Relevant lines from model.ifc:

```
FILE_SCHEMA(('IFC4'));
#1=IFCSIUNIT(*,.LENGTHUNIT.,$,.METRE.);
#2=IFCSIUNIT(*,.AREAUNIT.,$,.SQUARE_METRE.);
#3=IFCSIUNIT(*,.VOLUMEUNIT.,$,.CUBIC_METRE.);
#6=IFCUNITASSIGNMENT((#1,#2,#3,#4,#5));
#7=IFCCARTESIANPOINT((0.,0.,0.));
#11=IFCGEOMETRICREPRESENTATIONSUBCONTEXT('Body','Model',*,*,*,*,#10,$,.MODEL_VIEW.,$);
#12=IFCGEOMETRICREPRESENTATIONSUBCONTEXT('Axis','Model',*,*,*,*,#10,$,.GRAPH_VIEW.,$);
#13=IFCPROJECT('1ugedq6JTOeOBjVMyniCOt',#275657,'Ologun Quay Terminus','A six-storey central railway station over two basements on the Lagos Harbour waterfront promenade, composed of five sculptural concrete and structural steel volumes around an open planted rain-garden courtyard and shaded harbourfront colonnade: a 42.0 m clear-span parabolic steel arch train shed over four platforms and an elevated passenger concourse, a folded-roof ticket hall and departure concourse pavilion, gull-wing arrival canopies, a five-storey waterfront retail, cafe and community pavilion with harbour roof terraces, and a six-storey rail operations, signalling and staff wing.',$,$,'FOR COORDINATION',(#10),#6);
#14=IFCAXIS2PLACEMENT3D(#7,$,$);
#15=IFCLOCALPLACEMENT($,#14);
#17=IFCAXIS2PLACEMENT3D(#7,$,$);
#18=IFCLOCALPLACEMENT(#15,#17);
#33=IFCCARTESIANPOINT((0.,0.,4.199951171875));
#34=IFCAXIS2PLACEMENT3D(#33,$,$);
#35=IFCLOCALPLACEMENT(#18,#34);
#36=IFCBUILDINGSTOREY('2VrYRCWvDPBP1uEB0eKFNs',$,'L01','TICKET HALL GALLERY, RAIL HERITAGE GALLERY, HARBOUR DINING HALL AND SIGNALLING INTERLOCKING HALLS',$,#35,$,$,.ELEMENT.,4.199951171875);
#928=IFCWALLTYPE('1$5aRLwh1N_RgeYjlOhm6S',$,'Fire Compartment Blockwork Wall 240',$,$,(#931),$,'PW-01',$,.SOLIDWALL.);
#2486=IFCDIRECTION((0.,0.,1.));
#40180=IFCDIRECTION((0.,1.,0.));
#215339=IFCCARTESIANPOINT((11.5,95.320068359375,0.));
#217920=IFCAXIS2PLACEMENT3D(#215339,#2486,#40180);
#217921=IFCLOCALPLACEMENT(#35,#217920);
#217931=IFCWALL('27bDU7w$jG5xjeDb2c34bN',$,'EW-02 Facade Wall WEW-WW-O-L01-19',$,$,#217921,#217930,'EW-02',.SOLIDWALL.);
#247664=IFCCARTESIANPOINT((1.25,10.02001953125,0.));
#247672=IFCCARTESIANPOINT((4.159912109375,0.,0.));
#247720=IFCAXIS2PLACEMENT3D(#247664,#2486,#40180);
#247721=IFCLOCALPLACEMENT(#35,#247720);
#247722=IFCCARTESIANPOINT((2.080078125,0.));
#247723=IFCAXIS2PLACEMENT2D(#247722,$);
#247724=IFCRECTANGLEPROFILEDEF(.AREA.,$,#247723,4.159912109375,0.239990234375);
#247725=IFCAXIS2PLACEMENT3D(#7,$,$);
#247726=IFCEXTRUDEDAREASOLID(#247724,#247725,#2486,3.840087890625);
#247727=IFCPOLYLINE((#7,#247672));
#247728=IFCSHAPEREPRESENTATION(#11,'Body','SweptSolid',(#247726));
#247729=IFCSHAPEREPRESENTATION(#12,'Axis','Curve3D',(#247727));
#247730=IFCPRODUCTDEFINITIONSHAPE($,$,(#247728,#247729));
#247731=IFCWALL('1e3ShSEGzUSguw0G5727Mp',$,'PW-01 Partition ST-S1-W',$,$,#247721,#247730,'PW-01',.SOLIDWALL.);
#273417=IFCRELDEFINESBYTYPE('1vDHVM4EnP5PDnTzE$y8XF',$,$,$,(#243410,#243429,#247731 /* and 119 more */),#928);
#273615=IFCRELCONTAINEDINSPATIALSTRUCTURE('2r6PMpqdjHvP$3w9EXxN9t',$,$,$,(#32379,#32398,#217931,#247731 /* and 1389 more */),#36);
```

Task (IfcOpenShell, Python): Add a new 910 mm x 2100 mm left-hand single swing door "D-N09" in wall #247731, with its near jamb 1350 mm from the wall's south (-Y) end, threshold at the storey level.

```python
import numpy as np
import ifcopenshell
import ifcopenshell.api.feature
import ifcopenshell.api.geometry
import ifcopenshell.api.root
import ifcopenshell.api.spatial
import ifcopenshell.geom
import ifcopenshell.util.element
import ifcopenshell.util.placement
import ifcopenshell.util.representation
import ifcopenshell.util.shape
import ifcopenshell.util.unit

model = ifcopenshell.open("model.ifc")
unit_scale = ifcopenshell.util.unit.calculate_unit_scale(model)
settings = ifcopenshell.geom.settings()


def volume(element):
    """Net volume in cubic metres, openings subtracted."""
    shape = ifcopenshell.geom.create_shape(settings, element)
    return ifcopenshell.util.shape.get_volume(shape.geometry)


wall = model.by_guid("1e3ShSEGzUSguw0G5727Mp")
storey = ifcopenshell.util.element.get_container(wall, ifc_class="IfcBuildingStorey")
context = ifcopenshell.util.representation.get_context(model, "Model", "Body", "MODEL_VIEW")
before = volume(wall)

width, height, from_end, sill = 0.91, 2.1, 1.35, 0.0  # metres

# The wall runs along its own X axis, and the end named is its -X end.
wall_shape = ifcopenshell.geom.create_shape(settings, wall)
x, y, z = ifcopenshell.util.shape.get_vertices(wall_shape.geometry).T
start = x.min() + from_end
face, thickness = float(y.min()), float(y.max() - y.min())
wall_matrix = ifcopenshell.util.placement.get_local_placement(wall.ObjectPlacement)
level = ifcopenshell.util.placement.get_local_placement(storey.ObjectPlacement)[2, 3]


def in_wall(x, y):
    """Placement at x, y metres in the wall's axes, at sill height."""
    matrix = wall_matrix.copy()
    matrix[:, 3] = wall_matrix @ np.array([x / unit_scale, y / unit_scale, 0.0, 1.0])
    matrix[2, 3] = level + sill / unit_scale
    return matrix


# Opening: a box that overshoots both wall faces by 50 mm.
opening = ifcopenshell.api.root.create_entity(model, ifc_class="IfcOpeningElement", predefined_type="OPENING")
box = ifcopenshell.api.geometry.add_wall_representation(
    model, context=context, length=width, height=height, thickness=thickness + 0.1
)
ifcopenshell.api.geometry.assign_representation(model, product=opening, representation=box)
ifcopenshell.api.geometry.edit_object_placement(model, product=opening, matrix=in_wall(start, face - 0.05), is_si=False)
ifcopenshell.api.feature.add_feature(model, feature=opening, element=wall)

door = ifcopenshell.api.root.create_entity(model, ifc_class="IfcDoor", name="D-N09", predefined_type="DOOR")
door.OverallWidth, door.OverallHeight = width / unit_scale, height / unit_scale
door.OperationType = "SINGLE_SWING_LEFT"
body = ifcopenshell.api.geometry.add_door_representation(
    model,
    context=context,
    overall_width=door.OverallWidth,
    overall_height=door.OverallHeight,
    operation_type="SINGLE_SWING_LEFT",
    lining_properties={"LiningDepth": thickness / unit_scale, "ThresholdDepth": thickness / unit_scale},
)
ifcopenshell.api.geometry.assign_representation(model, product=door, representation=body)
ifcopenshell.api.spatial.assign_container(model, products=[door], relating_structure=storey)
ifcopenshell.api.feature.add_filling(model, opening=opening, element=door)

# The lining spans the wall, so the door starts at the wall face.
ifcopenshell.api.geometry.edit_object_placement(model, product=door, matrix=in_wall(start, face), is_si=False)

after = volume(wall)

print(f"wall volume {before:.3f} -> {after:.3f} m3")

model.write("model_v2.ifc")
```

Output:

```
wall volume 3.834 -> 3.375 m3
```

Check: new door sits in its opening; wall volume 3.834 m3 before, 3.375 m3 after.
